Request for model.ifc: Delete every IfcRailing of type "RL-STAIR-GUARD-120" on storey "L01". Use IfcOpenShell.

First a look at what the model holds.

```python
import ifcopenshell
import ifcopenshell.util.element

model = ifcopenshell.open("model.ifc")
print(model.schema)
storey = next(s for s in model.by_type("IfcBuildingStorey") if s.Name == "L01")
railings = [e for e in ifcopenshell.util.element.get_decomposition(storey) if e.is_a("IfcRailing")]
seen = {}
for e in railings:
    element_type = ifcopenshell.util.element.get_type(e)
    name = element_type.Name if element_type not in (None, e) else None
    seen[name] = seen.get(name, 0) + 1
for name, count in sorted(seen.items(), key=str):
    print(count, "x", name)
```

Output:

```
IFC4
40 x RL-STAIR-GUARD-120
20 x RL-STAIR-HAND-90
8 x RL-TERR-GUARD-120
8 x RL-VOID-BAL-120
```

```python
import ifcopenshell
import ifcopenshell.api.root
import ifcopenshell.util.element

model = ifcopenshell.open("model.ifc")

storey = next(s for s in model.by_type("IfcBuildingStorey") if s.Name == "L01")
railings = [e for e in ifcopenshell.util.element.get_decomposition(storey) if e.is_a("IfcRailing")]
targets = [e for e in railings if (t := ifcopenshell.util.element.get_type(e)) not in (None, e) and t.Name == "RL-STAIR-GUARD-120"]

for e in targets:
    ifcopenshell.api.root.remove_product(model, product=e)
print(len(targets), "removed")

model.write("model_rev.ifc")
```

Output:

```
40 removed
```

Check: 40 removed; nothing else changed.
